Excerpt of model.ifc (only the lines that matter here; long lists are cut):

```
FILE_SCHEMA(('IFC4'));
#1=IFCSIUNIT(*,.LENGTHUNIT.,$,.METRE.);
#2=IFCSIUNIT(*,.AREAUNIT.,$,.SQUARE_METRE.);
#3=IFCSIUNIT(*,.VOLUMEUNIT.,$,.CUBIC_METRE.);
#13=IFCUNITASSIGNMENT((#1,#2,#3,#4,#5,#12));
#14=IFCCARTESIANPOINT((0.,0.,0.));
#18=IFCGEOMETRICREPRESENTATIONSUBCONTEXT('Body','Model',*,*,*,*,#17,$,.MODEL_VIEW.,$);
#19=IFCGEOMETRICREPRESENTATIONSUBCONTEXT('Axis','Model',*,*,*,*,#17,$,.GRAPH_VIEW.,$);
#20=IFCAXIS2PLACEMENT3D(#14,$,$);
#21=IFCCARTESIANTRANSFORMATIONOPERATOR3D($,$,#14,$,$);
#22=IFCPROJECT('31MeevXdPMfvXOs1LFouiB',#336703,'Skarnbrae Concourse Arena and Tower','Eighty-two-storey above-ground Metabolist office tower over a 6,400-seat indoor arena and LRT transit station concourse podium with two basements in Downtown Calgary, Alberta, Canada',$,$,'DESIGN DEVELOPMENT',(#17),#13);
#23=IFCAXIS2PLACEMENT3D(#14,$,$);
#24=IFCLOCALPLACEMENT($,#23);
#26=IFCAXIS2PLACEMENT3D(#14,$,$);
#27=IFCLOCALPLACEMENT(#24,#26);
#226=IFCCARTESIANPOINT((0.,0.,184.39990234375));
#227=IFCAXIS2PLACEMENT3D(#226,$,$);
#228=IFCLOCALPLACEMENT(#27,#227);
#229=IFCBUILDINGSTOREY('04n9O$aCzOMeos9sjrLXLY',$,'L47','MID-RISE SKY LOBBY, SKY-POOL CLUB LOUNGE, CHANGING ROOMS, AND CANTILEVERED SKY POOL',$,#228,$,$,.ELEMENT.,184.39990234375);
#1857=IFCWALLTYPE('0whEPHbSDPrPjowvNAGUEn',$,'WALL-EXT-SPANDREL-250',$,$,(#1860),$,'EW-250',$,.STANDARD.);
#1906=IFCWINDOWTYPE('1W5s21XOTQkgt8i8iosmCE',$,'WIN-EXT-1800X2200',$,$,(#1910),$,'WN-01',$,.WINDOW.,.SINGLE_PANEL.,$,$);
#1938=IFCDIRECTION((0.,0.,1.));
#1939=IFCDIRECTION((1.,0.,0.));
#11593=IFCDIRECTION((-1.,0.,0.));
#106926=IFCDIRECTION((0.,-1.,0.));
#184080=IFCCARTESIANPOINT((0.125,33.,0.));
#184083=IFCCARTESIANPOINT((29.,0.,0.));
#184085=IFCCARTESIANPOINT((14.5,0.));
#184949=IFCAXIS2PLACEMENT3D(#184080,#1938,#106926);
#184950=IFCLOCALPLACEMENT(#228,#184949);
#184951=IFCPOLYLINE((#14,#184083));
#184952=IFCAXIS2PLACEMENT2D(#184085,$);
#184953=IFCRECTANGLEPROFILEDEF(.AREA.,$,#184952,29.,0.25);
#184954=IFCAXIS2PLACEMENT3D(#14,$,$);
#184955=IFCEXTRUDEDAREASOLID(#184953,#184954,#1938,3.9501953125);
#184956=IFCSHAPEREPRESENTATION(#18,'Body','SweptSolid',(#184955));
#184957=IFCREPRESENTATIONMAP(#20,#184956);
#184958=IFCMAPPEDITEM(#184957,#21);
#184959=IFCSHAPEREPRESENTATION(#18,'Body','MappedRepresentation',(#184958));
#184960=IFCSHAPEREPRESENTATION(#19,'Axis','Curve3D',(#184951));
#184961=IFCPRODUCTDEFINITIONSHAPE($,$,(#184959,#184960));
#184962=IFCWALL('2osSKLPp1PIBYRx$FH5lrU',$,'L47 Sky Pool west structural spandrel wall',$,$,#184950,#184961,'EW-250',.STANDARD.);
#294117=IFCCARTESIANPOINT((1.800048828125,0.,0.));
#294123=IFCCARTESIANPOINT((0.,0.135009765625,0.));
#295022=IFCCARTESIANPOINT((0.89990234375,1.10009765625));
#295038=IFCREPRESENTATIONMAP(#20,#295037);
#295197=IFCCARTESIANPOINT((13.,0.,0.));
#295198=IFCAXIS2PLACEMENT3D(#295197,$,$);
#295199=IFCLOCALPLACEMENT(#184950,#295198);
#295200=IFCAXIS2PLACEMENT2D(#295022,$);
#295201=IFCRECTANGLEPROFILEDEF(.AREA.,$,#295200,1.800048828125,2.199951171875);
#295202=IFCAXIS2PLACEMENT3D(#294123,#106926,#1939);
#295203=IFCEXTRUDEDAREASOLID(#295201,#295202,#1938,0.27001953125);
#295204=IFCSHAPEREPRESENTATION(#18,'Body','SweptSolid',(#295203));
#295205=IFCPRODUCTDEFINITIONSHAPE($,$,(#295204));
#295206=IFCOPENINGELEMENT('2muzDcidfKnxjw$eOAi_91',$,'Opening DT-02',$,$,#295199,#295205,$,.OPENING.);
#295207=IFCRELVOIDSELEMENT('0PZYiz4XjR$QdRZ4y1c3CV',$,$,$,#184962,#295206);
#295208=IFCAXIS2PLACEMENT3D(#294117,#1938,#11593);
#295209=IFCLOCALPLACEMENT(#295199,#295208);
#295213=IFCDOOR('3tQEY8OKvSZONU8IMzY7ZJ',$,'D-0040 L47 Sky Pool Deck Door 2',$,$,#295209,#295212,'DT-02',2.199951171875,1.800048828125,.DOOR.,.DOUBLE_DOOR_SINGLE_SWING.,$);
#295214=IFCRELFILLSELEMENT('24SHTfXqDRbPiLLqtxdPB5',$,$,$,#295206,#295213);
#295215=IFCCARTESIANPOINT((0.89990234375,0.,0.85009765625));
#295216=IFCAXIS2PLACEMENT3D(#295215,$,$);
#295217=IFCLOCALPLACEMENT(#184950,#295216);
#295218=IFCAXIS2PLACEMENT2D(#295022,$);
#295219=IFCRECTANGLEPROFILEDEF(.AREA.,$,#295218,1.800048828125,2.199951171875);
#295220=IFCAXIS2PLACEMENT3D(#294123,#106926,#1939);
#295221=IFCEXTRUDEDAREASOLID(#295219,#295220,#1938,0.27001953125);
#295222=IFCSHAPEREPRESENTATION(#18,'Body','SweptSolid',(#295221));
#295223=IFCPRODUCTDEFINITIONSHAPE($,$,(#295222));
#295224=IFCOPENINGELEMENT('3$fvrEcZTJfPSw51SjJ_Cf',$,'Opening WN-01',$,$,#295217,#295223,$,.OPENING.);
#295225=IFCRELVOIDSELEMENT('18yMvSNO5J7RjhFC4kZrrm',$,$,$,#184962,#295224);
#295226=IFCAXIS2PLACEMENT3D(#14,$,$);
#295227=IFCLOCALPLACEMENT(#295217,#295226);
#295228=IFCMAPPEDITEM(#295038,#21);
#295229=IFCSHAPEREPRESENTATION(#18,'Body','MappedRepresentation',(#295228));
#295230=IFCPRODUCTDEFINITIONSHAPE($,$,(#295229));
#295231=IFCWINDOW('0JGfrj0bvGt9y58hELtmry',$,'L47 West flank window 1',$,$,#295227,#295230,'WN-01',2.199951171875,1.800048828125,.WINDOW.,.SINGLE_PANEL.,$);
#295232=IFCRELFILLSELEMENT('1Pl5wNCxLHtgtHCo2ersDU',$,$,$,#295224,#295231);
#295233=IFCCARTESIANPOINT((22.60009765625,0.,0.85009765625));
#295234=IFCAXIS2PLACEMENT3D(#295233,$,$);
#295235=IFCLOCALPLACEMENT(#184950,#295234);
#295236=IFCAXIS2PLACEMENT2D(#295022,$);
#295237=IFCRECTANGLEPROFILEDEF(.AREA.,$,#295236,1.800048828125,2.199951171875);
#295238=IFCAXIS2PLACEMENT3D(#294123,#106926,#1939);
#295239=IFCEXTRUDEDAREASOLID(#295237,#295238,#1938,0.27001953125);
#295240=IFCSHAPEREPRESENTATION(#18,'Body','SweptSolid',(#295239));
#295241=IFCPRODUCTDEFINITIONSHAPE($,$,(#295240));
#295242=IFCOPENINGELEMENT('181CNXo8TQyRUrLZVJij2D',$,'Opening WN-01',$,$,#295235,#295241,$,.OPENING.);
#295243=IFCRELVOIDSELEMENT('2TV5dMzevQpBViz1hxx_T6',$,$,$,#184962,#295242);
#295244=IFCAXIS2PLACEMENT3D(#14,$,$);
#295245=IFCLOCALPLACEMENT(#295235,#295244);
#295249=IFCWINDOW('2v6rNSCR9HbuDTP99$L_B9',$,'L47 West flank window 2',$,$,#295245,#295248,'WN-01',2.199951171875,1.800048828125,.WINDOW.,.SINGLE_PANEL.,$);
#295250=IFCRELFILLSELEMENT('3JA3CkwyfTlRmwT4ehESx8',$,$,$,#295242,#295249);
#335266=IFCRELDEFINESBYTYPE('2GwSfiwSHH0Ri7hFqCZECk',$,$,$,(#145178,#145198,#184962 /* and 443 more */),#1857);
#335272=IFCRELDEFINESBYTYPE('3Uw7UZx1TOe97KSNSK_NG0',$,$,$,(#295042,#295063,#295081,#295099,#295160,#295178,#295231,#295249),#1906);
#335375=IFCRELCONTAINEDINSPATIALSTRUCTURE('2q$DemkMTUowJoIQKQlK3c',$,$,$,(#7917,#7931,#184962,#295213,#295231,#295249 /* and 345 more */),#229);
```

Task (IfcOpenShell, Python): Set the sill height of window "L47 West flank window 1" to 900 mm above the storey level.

```python
import numpy as np
import ifcopenshell
import ifcopenshell.api.geometry
import ifcopenshell.geom
import ifcopenshell.util.element
import ifcopenshell.util.placement
import ifcopenshell.util.shape
import ifcopenshell.util.unit

model = ifcopenshell.open("model.ifc")
unit_scale = ifcopenshell.util.unit.calculate_unit_scale(model)

window = model.by_guid("0JGfrj0bvGt9y58hELtmry")
opening = window.FillsVoids[0].RelatingOpeningElement
storey = ifcopenshell.util.element.get_container(window, ifc_class="IfcBuildingStorey")
level = ifcopenshell.util.placement.get_local_placement(storey.ObjectPlacement)[2, 3]

# The opening's origin need not be at the sill, so measure its lowest point.
shape = ifcopenshell.geom.create_shape(ifcopenshell.geom.settings(), opening)
bottom = ifcopenshell.util.shape.get_shape_bottom_elevation(shape, shape.geometry) / unit_scale
dz = level + 0.9 / unit_scale - bottom

shift = np.array([0.0, 0.0, dz])
# The window is placed relative to its opening, so it follows when the opening moves.
matrix = ifcopenshell.util.placement.get_local_placement(opening.ObjectPlacement)
matrix[:3, 3] += shift
ifcopenshell.api.geometry.edit_object_placement(
    model, product=opening, matrix=matrix, is_si=False, should_transform_children=True
)

print(f"moved by {dz * unit_scale:+.3f} m")

model.write("model_rev.ifc")
```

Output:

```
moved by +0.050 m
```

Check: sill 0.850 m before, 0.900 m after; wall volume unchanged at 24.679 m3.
